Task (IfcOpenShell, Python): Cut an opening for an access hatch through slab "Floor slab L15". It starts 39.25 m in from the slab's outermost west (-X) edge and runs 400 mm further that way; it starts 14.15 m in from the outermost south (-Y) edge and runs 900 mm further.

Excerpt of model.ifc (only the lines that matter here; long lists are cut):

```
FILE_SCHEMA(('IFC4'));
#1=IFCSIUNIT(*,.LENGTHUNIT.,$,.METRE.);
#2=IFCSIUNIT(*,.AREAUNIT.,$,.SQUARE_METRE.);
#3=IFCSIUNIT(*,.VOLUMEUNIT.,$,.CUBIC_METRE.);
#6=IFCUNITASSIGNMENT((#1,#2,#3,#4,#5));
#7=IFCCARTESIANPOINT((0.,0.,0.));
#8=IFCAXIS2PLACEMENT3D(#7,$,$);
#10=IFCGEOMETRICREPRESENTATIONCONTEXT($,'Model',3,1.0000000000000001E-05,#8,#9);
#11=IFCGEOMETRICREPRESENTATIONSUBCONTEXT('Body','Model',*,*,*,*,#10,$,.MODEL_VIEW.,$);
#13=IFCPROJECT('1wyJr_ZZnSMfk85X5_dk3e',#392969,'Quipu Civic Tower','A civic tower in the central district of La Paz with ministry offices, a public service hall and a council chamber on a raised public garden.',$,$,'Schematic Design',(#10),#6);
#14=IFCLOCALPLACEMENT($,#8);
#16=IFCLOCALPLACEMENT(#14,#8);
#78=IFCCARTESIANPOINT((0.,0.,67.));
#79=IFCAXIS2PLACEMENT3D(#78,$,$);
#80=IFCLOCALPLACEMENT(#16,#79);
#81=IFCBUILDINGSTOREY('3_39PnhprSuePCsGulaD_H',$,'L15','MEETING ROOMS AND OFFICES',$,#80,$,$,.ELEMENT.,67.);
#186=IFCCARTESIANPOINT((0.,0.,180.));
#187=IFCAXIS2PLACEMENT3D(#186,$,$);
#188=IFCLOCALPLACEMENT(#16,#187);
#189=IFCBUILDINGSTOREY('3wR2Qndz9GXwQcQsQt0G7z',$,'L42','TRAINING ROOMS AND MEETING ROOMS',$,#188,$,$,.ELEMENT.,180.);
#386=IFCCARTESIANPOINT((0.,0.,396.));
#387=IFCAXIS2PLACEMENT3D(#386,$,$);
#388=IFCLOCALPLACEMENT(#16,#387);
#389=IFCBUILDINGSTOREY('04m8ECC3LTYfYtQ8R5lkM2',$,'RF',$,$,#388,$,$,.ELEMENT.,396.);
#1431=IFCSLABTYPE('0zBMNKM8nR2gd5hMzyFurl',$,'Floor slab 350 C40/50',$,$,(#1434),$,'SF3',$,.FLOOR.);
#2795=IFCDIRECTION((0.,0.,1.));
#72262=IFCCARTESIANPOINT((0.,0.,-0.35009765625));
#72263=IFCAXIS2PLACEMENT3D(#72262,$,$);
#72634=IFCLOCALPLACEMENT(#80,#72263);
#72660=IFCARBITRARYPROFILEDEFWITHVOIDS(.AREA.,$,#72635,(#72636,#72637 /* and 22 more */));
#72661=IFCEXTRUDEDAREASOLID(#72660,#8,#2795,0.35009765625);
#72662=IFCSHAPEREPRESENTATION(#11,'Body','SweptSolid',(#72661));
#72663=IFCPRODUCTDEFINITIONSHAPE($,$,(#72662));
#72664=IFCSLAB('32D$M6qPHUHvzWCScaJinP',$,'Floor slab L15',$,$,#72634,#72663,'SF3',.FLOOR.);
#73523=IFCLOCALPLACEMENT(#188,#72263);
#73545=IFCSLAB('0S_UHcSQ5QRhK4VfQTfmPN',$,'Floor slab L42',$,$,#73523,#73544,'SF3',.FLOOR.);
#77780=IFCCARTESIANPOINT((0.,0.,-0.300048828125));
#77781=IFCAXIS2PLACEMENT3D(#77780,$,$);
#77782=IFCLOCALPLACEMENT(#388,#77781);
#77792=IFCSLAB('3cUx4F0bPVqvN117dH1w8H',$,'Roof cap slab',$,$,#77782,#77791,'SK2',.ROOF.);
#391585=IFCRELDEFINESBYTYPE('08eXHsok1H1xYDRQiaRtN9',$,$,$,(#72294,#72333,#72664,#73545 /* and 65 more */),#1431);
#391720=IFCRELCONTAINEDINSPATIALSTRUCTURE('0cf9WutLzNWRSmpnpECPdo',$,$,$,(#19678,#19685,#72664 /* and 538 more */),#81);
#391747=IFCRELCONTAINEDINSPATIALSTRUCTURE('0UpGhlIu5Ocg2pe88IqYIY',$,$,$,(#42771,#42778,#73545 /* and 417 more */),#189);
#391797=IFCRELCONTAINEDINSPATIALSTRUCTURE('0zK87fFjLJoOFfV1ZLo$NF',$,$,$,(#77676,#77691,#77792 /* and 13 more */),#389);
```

```python
import numpy as np
import ifcopenshell
import ifcopenshell.api.feature
import ifcopenshell.api.geometry
import ifcopenshell.api.root
import ifcopenshell.geom
import ifcopenshell.util.placement
import ifcopenshell.util.representation
import ifcopenshell.util.shape
import ifcopenshell.util.unit

model = ifcopenshell.open("model.ifc")
unit_scale = ifcopenshell.util.unit.calculate_unit_scale(model)
settings = ifcopenshell.geom.settings()


def volume(element):
    """Net volume in cubic metres, openings subtracted."""
    shape = ifcopenshell.geom.create_shape(settings, element)
    return ifcopenshell.util.shape.get_volume(shape.geometry)


slab = model.by_id(72664)
before = volume(slab)

# Extent in the slab's own axes, in metres. The edges named are its -X and -Y sides.
slab_shape = ifcopenshell.geom.create_shape(settings, slab)
vertices = ifcopenshell.util.shape.get_vertices(slab_shape.geometry)
x_min, y_min, bottom = vertices.min(axis=0)
top = vertices[:, 2].max()

opening = ifcopenshell.api.root.create_entity(model, ifc_class="IfcOpeningElement", name="Access hatch opening", predefined_type="OPENING")
context = ifcopenshell.util.representation.get_context(model, "Model", "Body", "MODEL_VIEW")
width, depth = 0.4, 0.9
outline = [(0.0, 0.0), (width, 0.0), (width, depth), (0.0, depth), (0.0, 0.0)]
# Overshoot both faces by 50 mm so the cut is clean.
shape = ifcopenshell.api.geometry.add_slab_representation(
    model, context=context, depth=top - bottom + 0.1, polyline=outline
)
ifcopenshell.api.geometry.assign_representation(model, product=opening, representation=shape)

matrix = ifcopenshell.util.placement.get_local_placement(slab.ObjectPlacement)
matrix[:, 3] = matrix @ np.append(np.array([x_min + 39.25, y_min + 14.15, bottom - 0.05]) / unit_scale, 1.0)
ifcopenshell.api.geometry.edit_object_placement(model, product=opening, matrix=matrix, is_si=False)
ifcopenshell.api.feature.add_feature(model, feature=opening, element=slab)

after = volume(slab)

print(f"slab volume {before:.3f} -> {after:.3f} m3")

model.write("model_edited.ifc")
```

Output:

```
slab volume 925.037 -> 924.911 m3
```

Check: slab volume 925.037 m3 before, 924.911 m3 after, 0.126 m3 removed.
